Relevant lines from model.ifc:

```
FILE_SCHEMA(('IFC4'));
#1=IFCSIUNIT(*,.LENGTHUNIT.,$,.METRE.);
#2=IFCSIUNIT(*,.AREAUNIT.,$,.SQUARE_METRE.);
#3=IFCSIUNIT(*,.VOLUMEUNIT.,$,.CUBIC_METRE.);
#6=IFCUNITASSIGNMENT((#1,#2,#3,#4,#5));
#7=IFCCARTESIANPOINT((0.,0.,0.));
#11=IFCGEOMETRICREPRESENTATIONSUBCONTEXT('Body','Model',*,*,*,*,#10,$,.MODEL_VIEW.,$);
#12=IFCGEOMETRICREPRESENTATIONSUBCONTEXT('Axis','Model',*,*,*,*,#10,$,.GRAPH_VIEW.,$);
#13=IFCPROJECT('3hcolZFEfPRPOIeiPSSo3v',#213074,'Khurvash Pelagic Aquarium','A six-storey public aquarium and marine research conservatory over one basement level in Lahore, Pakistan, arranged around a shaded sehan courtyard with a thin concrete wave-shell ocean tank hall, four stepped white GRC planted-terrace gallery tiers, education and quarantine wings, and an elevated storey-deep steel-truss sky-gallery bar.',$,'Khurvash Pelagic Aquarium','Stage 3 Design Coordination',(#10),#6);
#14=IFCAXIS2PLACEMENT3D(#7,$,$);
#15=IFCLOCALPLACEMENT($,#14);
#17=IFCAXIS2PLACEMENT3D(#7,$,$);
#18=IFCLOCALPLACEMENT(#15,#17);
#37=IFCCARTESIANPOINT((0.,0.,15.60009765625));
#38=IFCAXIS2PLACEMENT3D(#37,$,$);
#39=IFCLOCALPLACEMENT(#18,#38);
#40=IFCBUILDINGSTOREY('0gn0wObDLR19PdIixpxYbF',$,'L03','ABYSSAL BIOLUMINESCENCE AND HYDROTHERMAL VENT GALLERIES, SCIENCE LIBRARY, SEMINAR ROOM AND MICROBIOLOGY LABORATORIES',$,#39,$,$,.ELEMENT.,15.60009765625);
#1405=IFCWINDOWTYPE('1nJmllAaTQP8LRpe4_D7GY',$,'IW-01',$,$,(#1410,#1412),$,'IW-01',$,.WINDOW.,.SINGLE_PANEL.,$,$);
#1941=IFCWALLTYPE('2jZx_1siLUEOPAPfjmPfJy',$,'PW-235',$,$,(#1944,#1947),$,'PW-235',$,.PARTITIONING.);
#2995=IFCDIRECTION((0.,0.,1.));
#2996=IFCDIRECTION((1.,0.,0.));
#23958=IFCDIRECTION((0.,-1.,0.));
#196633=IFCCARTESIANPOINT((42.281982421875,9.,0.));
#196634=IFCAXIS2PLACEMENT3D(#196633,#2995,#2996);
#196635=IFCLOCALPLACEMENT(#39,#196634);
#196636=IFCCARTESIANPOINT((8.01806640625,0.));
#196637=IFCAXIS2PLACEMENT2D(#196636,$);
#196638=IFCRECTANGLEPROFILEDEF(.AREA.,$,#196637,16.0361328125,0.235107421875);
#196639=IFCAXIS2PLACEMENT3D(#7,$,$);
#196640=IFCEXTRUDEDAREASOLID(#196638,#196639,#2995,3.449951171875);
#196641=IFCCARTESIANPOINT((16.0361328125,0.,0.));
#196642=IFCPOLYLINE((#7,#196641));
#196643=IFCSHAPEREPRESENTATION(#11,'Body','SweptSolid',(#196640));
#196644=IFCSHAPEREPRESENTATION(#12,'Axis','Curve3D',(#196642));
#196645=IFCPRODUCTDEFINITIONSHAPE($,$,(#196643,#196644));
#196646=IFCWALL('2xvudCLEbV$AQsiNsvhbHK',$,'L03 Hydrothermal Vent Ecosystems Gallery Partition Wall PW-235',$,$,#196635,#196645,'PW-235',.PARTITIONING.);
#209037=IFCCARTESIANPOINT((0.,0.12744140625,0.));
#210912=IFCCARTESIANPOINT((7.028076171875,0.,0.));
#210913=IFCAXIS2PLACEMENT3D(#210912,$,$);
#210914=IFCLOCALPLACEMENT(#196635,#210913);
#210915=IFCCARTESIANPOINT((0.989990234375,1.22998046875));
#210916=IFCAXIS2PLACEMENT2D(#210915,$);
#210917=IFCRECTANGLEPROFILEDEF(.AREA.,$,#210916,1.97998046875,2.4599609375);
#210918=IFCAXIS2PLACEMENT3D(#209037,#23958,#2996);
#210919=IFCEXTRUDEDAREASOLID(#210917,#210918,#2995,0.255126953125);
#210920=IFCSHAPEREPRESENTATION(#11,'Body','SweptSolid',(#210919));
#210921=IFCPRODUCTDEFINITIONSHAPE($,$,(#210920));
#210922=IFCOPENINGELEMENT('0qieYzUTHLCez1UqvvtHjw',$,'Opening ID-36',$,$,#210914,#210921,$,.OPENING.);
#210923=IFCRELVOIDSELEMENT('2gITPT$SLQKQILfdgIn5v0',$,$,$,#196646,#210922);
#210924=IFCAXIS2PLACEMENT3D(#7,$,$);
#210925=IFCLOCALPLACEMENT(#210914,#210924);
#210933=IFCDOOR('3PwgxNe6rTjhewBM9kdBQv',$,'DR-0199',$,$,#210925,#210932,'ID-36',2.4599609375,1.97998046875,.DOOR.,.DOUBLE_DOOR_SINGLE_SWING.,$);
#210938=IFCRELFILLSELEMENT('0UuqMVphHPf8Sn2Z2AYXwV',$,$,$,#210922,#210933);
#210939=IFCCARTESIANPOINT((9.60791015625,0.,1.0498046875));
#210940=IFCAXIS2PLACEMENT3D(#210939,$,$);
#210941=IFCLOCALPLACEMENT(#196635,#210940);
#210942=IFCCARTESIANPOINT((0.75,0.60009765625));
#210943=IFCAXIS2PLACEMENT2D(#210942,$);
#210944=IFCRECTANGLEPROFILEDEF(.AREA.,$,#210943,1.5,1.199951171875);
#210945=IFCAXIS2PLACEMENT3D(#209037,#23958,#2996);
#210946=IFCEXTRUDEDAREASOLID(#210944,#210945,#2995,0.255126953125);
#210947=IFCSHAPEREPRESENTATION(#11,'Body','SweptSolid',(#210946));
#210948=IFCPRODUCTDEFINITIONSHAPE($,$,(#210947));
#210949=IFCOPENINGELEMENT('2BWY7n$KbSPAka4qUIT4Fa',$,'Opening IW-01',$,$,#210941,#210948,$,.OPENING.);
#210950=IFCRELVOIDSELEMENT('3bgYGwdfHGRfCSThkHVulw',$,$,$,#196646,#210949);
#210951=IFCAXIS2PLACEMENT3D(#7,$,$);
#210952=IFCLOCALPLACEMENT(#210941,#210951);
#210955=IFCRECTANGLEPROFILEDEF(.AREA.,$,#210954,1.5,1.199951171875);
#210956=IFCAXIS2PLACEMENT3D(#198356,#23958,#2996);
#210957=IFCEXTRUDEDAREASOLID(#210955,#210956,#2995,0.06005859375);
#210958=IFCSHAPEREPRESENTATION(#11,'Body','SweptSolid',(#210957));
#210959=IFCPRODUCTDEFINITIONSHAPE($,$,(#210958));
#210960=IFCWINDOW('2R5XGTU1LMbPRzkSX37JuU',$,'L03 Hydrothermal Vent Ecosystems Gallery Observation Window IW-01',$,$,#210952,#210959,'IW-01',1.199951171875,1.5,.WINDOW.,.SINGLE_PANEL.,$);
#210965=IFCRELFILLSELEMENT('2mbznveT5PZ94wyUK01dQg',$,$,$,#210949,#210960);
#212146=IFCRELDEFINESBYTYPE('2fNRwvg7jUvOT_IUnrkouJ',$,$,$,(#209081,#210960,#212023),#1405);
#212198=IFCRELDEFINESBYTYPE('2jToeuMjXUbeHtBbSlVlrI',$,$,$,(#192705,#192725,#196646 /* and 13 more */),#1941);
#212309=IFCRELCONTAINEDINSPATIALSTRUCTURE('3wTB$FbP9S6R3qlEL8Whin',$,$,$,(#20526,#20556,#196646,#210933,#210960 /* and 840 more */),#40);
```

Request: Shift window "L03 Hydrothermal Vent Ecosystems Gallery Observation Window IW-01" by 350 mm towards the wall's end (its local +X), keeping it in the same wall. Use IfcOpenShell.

```python
import ifcopenshell
import ifcopenshell.api.geometry
import ifcopenshell.util.placement

model = ifcopenshell.open("model.ifc")

window = model.by_guid("2R5XGTU1LMbPRzkSX37JuU")
opening = window.FillsVoids[0].RelatingOpeningElement
wall = opening.VoidsElements[0].RelatingBuildingElement

wall_matrix = ifcopenshell.util.placement.get_local_placement(wall.ObjectPlacement)
shift = wall_matrix[:3, 0] * 0.35
before = ifcopenshell.util.placement.get_local_placement(window.ObjectPlacement)[:3, 3].copy()

# The window is placed relative to its opening, so it follows when the opening moves.
matrix = ifcopenshell.util.placement.get_local_placement(opening.ObjectPlacement)
matrix[:3, 3] += shift
ifcopenshell.api.geometry.edit_object_placement(
    model, product=opening, matrix=matrix, is_si=False, should_transform_children=True
)

after = ifcopenshell.util.placement.get_local_placement(window.ObjectPlacement)[:3, 3]
print("window moved by", (after - before).round(3) + 0.0)

model.write("model_v2.ifc")
```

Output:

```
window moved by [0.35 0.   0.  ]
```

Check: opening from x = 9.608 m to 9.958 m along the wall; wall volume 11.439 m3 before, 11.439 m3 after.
